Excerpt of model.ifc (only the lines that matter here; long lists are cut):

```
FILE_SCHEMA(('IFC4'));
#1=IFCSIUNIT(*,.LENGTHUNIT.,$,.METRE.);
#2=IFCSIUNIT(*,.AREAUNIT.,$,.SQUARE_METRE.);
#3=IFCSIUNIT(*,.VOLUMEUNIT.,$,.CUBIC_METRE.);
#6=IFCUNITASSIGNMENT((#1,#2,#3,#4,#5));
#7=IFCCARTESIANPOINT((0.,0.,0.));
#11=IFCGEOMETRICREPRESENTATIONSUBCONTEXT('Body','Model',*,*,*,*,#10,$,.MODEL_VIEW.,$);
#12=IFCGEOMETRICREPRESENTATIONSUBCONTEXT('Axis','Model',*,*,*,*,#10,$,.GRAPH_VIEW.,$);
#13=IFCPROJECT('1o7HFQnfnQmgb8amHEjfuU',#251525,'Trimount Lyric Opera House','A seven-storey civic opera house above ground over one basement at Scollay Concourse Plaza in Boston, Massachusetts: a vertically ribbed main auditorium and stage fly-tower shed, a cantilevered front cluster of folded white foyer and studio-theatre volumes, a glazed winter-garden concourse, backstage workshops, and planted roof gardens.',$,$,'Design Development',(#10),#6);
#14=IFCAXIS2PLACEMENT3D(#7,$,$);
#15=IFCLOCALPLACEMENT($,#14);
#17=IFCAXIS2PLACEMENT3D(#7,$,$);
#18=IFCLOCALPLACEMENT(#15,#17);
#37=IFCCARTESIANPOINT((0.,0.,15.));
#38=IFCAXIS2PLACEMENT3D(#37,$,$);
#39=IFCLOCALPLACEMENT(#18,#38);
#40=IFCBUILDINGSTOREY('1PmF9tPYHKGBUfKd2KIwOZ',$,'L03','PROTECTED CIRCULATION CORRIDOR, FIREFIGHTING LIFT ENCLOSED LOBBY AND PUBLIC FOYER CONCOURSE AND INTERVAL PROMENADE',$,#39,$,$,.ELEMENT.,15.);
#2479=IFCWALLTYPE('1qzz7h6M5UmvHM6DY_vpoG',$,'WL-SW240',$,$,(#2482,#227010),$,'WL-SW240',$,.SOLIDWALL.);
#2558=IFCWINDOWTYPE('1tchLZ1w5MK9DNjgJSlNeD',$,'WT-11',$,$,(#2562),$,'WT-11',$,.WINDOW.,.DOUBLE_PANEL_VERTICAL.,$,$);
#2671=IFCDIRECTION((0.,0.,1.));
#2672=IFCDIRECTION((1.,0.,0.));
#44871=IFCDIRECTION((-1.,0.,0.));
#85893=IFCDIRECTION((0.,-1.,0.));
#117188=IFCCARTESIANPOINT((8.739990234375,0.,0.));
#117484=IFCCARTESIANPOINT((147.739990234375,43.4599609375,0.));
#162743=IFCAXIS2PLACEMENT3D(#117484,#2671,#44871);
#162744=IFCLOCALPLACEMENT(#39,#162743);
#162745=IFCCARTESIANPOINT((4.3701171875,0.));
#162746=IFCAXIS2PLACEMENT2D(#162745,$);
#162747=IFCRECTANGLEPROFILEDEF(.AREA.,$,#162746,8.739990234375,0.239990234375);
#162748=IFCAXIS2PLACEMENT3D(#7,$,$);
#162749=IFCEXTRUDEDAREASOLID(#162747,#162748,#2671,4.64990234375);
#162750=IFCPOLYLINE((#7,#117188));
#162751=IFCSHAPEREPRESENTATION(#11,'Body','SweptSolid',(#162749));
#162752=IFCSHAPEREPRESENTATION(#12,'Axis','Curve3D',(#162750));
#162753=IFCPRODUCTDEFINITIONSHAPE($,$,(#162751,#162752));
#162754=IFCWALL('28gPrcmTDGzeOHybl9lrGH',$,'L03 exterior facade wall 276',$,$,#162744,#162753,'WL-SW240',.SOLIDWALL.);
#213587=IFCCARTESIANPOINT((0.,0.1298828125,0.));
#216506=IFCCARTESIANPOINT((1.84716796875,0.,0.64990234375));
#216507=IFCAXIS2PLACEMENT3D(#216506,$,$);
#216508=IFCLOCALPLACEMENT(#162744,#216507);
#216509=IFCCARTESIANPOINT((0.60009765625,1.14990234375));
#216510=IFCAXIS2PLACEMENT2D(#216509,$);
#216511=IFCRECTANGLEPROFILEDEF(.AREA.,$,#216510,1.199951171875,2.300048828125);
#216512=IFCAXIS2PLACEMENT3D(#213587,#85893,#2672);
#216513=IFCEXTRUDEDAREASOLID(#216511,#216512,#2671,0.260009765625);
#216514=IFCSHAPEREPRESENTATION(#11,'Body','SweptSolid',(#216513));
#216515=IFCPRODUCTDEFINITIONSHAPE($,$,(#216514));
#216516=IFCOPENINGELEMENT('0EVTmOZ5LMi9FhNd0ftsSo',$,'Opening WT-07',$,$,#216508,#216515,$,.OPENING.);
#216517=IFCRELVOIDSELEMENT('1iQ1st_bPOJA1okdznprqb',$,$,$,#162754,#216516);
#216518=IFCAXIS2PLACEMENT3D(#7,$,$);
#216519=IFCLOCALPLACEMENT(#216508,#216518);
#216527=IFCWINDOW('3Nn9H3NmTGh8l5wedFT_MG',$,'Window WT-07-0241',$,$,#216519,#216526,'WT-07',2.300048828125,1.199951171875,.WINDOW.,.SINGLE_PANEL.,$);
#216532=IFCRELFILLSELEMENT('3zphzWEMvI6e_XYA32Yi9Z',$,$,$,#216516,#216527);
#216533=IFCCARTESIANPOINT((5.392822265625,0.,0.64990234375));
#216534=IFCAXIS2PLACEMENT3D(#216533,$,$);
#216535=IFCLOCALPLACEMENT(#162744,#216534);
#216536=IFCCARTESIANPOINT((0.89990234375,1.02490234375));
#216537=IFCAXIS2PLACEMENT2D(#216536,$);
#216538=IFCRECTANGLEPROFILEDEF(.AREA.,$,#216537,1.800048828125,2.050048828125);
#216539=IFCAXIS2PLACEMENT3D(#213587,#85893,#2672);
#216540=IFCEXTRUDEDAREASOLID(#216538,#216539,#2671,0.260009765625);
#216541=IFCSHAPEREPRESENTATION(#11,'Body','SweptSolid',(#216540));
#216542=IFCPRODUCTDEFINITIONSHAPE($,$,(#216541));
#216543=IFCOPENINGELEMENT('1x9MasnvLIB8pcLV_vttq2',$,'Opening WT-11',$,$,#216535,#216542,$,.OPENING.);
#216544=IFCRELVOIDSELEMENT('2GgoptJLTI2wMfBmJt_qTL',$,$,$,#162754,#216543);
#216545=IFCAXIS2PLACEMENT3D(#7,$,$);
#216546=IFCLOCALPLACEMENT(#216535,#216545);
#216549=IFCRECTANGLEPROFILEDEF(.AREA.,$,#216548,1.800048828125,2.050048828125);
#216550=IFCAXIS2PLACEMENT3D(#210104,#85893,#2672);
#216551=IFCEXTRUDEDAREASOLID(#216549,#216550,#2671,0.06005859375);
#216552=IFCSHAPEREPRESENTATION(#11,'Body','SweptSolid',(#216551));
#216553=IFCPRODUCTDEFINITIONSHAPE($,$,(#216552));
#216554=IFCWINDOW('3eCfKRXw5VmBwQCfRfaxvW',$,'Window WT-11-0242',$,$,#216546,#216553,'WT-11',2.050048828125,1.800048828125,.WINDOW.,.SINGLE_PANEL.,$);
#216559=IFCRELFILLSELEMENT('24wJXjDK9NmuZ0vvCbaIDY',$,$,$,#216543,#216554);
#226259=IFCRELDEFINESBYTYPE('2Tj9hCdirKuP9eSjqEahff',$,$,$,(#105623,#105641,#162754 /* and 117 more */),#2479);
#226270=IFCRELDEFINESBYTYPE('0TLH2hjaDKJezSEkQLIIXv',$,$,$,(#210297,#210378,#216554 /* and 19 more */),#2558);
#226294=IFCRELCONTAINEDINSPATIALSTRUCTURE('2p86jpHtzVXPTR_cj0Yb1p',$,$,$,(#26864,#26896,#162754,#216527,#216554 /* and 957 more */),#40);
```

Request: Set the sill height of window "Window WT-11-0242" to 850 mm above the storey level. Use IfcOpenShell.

```python
import numpy as np
import ifcopenshell
import ifcopenshell.api.geometry
import ifcopenshell.geom
import ifcopenshell.util.element
import ifcopenshell.util.placement
import ifcopenshell.util.shape
import ifcopenshell.util.unit

model = ifcopenshell.open("model.ifc")
unit_scale = ifcopenshell.util.unit.calculate_unit_scale(model)

window = model.by_id(216554)
opening = window.FillsVoids[0].RelatingOpeningElement
storey = ifcopenshell.util.element.get_container(window, ifc_class="IfcBuildingStorey")
level = ifcopenshell.util.placement.get_local_placement(storey.ObjectPlacement)[2, 3]

# The opening's origin need not be at the sill, so measure its lowest point.
shape = ifcopenshell.geom.create_shape(ifcopenshell.geom.settings(), opening)
bottom = ifcopenshell.util.shape.get_shape_bottom_elevation(shape, shape.geometry) / unit_scale
dz = level + 0.85 / unit_scale - bottom

shift = np.array([0.0, 0.0, dz])
# The window is placed relative to its opening, so it follows when the opening moves.
matrix = ifcopenshell.util.placement.get_local_placement(opening.ObjectPlacement)
matrix[:3, 3] += shift
ifcopenshell.api.geometry.edit_object_placement(
    model, product=opening, matrix=matrix, is_si=False, should_transform_children=True
)

print(f"moved by {dz * unit_scale:+.3f} m")

model.write("model_edited.ifc")
```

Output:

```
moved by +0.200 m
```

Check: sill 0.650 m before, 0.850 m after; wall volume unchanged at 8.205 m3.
